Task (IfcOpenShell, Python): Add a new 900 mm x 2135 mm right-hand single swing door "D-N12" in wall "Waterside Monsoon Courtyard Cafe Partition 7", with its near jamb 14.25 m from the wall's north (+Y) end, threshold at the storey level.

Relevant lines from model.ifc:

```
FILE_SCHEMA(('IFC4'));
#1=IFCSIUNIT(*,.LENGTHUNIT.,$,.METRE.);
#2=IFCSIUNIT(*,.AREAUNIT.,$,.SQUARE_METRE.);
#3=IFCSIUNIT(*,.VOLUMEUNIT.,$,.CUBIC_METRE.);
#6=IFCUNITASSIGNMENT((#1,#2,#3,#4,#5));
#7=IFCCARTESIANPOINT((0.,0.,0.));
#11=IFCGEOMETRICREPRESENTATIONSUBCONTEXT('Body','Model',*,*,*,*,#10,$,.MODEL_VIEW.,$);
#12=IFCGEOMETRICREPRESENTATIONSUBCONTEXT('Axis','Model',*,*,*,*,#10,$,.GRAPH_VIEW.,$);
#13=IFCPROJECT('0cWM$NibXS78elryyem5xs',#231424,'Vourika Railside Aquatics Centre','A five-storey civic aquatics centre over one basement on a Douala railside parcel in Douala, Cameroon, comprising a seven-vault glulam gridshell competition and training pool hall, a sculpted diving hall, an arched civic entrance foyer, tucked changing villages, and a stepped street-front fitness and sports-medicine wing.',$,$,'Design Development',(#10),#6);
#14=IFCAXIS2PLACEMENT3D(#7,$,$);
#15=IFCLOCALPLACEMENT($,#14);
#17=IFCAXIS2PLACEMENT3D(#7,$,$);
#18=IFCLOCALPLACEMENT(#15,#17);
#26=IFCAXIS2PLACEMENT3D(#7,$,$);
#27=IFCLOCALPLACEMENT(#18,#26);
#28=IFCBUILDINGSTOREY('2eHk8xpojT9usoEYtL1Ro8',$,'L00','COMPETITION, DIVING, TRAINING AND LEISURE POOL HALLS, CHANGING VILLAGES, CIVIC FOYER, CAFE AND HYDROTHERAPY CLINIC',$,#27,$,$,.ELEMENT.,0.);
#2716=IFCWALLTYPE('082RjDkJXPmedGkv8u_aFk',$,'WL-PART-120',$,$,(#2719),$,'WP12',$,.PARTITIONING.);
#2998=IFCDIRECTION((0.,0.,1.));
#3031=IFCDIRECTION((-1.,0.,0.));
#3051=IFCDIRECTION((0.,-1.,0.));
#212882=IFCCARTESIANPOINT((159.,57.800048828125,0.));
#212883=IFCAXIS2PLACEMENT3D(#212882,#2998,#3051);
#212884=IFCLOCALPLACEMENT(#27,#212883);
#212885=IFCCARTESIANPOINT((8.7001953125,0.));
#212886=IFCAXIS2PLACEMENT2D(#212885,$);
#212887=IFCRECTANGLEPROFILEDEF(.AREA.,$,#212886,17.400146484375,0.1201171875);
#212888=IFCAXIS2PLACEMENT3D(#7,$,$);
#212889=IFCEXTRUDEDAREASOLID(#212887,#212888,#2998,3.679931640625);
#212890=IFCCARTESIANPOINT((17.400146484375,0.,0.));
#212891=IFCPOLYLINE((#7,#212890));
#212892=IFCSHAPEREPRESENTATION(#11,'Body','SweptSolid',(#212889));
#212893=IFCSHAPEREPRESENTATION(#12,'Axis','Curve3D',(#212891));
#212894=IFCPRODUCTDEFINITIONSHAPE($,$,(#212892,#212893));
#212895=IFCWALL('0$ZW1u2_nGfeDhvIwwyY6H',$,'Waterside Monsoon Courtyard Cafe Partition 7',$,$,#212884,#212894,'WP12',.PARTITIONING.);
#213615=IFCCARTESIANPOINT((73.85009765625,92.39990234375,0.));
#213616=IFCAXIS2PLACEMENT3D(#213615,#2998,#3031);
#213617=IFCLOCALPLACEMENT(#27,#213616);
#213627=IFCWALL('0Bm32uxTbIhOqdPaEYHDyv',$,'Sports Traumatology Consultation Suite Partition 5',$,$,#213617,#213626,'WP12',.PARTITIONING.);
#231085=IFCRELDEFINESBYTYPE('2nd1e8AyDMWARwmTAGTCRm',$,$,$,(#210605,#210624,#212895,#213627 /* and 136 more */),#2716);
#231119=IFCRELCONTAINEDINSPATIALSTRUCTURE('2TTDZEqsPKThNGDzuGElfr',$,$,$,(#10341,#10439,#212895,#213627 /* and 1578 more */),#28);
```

```python
import numpy as np
import ifcopenshell
import ifcopenshell.api.feature
import ifcopenshell.api.geometry
import ifcopenshell.api.root
import ifcopenshell.api.spatial
import ifcopenshell.geom
import ifcopenshell.util.element
import ifcopenshell.util.placement
import ifcopenshell.util.representation
import ifcopenshell.util.shape
import ifcopenshell.util.unit

model = ifcopenshell.open("model.ifc")
unit_scale = ifcopenshell.util.unit.calculate_unit_scale(model)
settings = ifcopenshell.geom.settings()


def volume(element):
    """Net volume in cubic metres, openings subtracted."""
    shape = ifcopenshell.geom.create_shape(settings, element)
    return ifcopenshell.util.shape.get_volume(shape.geometry)


wall = model.by_guid("0$ZW1u2_nGfeDhvIwwyY6H")
storey = ifcopenshell.util.element.get_container(wall, ifc_class="IfcBuildingStorey")
context = ifcopenshell.util.representation.get_context(model, "Model", "Body", "MODEL_VIEW")
before = volume(wall)

width, height, from_end, sill = 0.9, 2.135, 14.25, 0.0  # metres

# The wall runs along its own X axis, and the end named is its -X end.
wall_shape = ifcopenshell.geom.create_shape(settings, wall)
x, y, z = ifcopenshell.util.shape.get_vertices(wall_shape.geometry).T
start = x.min() + from_end
face, thickness = float(y.min()), float(y.max() - y.min())
wall_matrix = ifcopenshell.util.placement.get_local_placement(wall.ObjectPlacement)
level = ifcopenshell.util.placement.get_local_placement(storey.ObjectPlacement)[2, 3]


def in_wall(x, y):
    """Placement at x, y metres in the wall's axes, at sill height."""
    matrix = wall_matrix.copy()
    matrix[:, 3] = wall_matrix @ np.array([x / unit_scale, y / unit_scale, 0.0, 1.0])
    matrix[2, 3] = level + sill / unit_scale
    return matrix


# Opening: a box that overshoots both wall faces by 50 mm.
opening = ifcopenshell.api.root.create_entity(model, ifc_class="IfcOpeningElement", predefined_type="OPENING")
box = ifcopenshell.api.geometry.add_wall_representation(
    model, context=context, length=width, height=height, thickness=thickness + 0.1
)
ifcopenshell.api.geometry.assign_representation(model, product=opening, representation=box)
ifcopenshell.api.geometry.edit_object_placement(model, product=opening, matrix=in_wall(start, face - 0.05), is_si=False)
ifcopenshell.api.feature.add_feature(model, feature=opening, element=wall)

door = ifcopenshell.api.root.create_entity(model, ifc_class="IfcDoor", name="D-N12", predefined_type="DOOR")
door.OverallWidth, door.OverallHeight = width / unit_scale, height / unit_scale
door.OperationType = "SINGLE_SWING_RIGHT"
body = ifcopenshell.api.geometry.add_door_representation(
    model,
    context=context,
    overall_width=door.OverallWidth,
    overall_height=door.OverallHeight,
    operation_type="SINGLE_SWING_RIGHT",
    lining_properties={"LiningDepth": thickness / unit_scale, "ThresholdDepth": thickness / unit_scale},
)
ifcopenshell.api.geometry.assign_representation(model, product=door, representation=body)
ifcopenshell.api.spatial.assign_container(model, products=[door], relating_structure=storey)
ifcopenshell.api.feature.add_filling(model, opening=opening, element=door)

# The lining spans the wall, so the door starts at the wall face.
ifcopenshell.api.geometry.edit_object_placement(model, product=door, matrix=in_wall(start, face), is_si=False)

after = volume(wall)

print(f"wall volume {before:.3f} -> {after:.3f} m3")

model.write("model-out.ifc")
```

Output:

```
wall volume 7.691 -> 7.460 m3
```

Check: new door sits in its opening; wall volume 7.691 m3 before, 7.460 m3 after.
